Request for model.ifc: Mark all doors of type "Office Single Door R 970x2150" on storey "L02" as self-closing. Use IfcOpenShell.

First a look at what the model holds.

```python
import ifcopenshell
import ifcopenshell.util.element

model = ifcopenshell.open("model.ifc")
print(model.schema)
storey = next(s for s in model.by_type("IfcBuildingStorey") if s.Name == "L02")
doors = [e for e in ifcopenshell.util.element.get_decomposition(storey) if e.is_a("IfcDoor")]
seen = {}
for e in doors:
    element_type = ifcopenshell.util.element.get_type(e)
    key = (element_type.Name if element_type != e and element_type else None, ifcopenshell.util.element.get_pset(e, "Pset_DoorCommon", "SelfClosing"))
    seen[key] = seen.get(key, 0) + 1
for (name, value), count in sorted(seen.items(), key=str):
    print(count, "x", name, "|", value)
```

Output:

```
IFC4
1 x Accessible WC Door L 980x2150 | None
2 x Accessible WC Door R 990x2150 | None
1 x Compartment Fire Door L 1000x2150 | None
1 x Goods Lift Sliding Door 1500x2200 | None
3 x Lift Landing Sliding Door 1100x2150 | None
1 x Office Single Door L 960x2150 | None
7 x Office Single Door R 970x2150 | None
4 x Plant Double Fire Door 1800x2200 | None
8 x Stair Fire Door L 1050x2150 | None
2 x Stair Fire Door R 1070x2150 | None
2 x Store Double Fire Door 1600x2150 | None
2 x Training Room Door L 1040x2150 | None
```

```python
import ifcopenshell
import ifcopenshell.api.pset
import ifcopenshell.util.element

model = ifcopenshell.open("model.ifc")

storey = next(s for s in model.by_type("IfcBuildingStorey") if s.Name == "L02")
doors = [e for e in ifcopenshell.util.element.get_decomposition(storey) if e.is_a("IfcDoor")]

count = 0
for e in doors:
    element_type = ifcopenshell.util.element.get_type(e)
    if element_type in (None, e) or element_type.Name != "Office Single Door R 970x2150":
        continue
    # add_pset returns the element's existing set when there is one.
    pset = ifcopenshell.api.pset.add_pset(model, product=e, name="Pset_DoorCommon")
    ifcopenshell.api.pset.edit_pset(model, pset=pset, properties={"SelfClosing": True})
    count += 1

print(count, "doors updated")

model.write("model_updated.ifc")
```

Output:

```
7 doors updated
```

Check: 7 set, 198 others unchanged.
